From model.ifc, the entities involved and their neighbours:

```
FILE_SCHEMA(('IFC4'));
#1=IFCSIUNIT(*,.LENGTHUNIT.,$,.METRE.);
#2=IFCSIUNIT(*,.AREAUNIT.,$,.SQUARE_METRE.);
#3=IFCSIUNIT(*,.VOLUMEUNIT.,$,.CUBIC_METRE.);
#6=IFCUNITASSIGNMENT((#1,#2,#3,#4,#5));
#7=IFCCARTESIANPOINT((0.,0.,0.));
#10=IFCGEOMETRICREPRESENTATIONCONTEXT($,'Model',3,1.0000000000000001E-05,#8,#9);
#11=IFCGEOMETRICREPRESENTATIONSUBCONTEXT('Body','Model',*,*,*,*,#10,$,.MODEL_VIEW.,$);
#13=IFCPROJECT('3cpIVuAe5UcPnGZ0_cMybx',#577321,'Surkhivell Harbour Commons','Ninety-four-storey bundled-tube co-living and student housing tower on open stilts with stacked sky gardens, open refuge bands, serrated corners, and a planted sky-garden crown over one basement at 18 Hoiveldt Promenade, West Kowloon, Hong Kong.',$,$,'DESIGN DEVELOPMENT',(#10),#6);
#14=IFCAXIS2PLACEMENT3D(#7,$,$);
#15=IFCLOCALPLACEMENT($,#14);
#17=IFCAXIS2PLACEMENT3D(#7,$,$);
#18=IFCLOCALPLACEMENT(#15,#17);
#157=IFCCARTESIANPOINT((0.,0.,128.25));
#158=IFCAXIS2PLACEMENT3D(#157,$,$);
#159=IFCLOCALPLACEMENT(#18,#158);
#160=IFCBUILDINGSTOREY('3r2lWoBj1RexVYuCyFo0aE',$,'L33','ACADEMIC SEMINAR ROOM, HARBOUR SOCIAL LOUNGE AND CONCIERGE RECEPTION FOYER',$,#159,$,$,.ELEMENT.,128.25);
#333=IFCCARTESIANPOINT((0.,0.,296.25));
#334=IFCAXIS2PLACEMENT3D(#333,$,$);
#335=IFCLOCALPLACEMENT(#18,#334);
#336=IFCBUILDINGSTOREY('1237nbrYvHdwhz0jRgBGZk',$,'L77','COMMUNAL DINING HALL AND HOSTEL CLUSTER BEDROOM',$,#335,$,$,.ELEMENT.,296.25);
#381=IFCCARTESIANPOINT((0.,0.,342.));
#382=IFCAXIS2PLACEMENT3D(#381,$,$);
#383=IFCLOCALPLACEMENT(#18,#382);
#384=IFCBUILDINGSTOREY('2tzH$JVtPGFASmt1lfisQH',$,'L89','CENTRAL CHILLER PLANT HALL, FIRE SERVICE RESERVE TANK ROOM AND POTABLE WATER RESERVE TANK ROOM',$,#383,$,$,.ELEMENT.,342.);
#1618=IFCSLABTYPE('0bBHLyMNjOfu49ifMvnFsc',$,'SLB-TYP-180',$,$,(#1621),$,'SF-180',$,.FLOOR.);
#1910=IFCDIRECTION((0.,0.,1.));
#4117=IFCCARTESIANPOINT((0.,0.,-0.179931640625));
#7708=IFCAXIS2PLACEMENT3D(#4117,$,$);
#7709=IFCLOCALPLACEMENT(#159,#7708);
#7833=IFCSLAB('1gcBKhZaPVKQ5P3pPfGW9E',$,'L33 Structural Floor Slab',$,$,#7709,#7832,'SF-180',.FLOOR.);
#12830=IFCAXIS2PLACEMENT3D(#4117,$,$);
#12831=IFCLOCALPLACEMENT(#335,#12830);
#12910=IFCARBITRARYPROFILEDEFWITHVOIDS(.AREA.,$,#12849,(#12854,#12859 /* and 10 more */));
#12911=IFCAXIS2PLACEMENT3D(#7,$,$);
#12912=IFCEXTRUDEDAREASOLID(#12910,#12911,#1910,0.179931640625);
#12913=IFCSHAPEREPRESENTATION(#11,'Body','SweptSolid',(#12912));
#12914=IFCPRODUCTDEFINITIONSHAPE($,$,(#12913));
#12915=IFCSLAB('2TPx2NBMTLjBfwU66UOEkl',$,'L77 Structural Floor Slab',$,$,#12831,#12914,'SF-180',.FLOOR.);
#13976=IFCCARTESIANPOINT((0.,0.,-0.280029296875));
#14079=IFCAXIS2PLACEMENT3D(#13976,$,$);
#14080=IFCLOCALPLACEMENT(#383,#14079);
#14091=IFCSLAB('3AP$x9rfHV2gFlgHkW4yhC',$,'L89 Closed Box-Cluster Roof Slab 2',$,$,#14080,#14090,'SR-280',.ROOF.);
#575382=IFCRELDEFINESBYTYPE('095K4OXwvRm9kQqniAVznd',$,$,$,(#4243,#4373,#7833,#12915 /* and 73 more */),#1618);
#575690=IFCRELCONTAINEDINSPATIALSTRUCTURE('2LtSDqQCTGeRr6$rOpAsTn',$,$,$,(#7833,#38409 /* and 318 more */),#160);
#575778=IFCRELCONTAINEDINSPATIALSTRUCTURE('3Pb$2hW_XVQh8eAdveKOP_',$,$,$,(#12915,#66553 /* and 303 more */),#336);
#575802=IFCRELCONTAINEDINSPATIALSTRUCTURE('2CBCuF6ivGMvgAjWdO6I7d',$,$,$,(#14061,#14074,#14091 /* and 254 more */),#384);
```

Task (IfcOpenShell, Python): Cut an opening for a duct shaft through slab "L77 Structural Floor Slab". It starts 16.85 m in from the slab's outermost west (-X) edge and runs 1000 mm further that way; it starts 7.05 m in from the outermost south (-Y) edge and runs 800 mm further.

```python
import numpy as np
import ifcopenshell
import ifcopenshell.api.feature
import ifcopenshell.api.geometry
import ifcopenshell.api.root
import ifcopenshell.geom
import ifcopenshell.util.placement
import ifcopenshell.util.representation
import ifcopenshell.util.shape
import ifcopenshell.util.unit

model = ifcopenshell.open("model.ifc")
unit_scale = ifcopenshell.util.unit.calculate_unit_scale(model)
settings = ifcopenshell.geom.settings()


def volume(element):
    """Net volume in cubic metres, openings subtracted."""
    shape = ifcopenshell.geom.create_shape(settings, element)
    return ifcopenshell.util.shape.get_volume(shape.geometry)


slab = model.by_guid("2TPx2NBMTLjBfwU66UOEkl")
before = volume(slab)

# Extent in the slab's own axes, in metres. The edges named are its -X and -Y sides.
slab_shape = ifcopenshell.geom.create_shape(settings, slab)
vertices = ifcopenshell.util.shape.get_vertices(slab_shape.geometry)
x_min, y_min, bottom = vertices.min(axis=0)
top = vertices[:, 2].max()

opening = ifcopenshell.api.root.create_entity(model, ifc_class="IfcOpeningElement", name="Duct shaft opening", predefined_type="OPENING")
context = ifcopenshell.util.representation.get_context(model, "Model", "Body", "MODEL_VIEW")
width, depth = 1, 0.8
outline = [(0.0, 0.0), (width, 0.0), (width, depth), (0.0, depth), (0.0, 0.0)]
# Overshoot both faces by 50 mm so the cut is clean.
shape = ifcopenshell.api.geometry.add_slab_representation(
    model, context=context, depth=top - bottom + 0.1, polyline=outline
)
ifcopenshell.api.geometry.assign_representation(model, product=opening, representation=shape)

matrix = ifcopenshell.util.placement.get_local_placement(slab.ObjectPlacement)
matrix[:, 3] = matrix @ np.append(np.array([x_min + 16.85, y_min + 7.05, bottom - 0.05]) / unit_scale, 1.0)
ifcopenshell.api.geometry.edit_object_placement(model, product=opening, matrix=matrix, is_si=False)
ifcopenshell.api.feature.add_feature(model, feature=opening, element=slab)

after = volume(slab)

print(f"slab volume {before:.3f} -> {after:.3f} m3")

model.write("model-out.ifc")
```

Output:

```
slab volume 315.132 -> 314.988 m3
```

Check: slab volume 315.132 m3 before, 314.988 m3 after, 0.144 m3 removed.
